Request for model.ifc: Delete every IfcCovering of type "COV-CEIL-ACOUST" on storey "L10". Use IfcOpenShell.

First a look at what the model holds.

```python
import ifcopenshell
import ifcopenshell.util.element

model = ifcopenshell.open("model.ifc")
print(model.schema)
storey = next(s for s in model.by_type("IfcBuildingStorey") if s.Name == "L10")
coverings = [e for e in ifcopenshell.util.element.get_decomposition(storey) if e.is_a("IfcCovering")]
seen = {}
for e in coverings:
    element_type = ifcopenshell.util.element.get_type(e)
    name = element_type.Name if element_type not in (None, e) else None
    seen[name] = seen.get(name, 0) + 1
for name, count in sorted(seen.items(), key=str):
    print(count, "x", name)
```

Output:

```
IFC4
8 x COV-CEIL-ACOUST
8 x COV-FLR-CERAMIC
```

```python
import ifcopenshell
import ifcopenshell.api.root
import ifcopenshell.util.element

model = ifcopenshell.open("model.ifc")

storey = next(s for s in model.by_type("IfcBuildingStorey") if s.Name == "L10")
coverings = [e for e in ifcopenshell.util.element.get_decomposition(storey) if e.is_a("IfcCovering")]
targets = [e for e in coverings if (t := ifcopenshell.util.element.get_type(e)) not in (None, e) and t.Name == "COV-CEIL-ACOUST"]

for e in targets:
    ifcopenshell.api.root.remove_product(model, product=e)
print(len(targets), "removed")

model.write("model_updated.ifc")
```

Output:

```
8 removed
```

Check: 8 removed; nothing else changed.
